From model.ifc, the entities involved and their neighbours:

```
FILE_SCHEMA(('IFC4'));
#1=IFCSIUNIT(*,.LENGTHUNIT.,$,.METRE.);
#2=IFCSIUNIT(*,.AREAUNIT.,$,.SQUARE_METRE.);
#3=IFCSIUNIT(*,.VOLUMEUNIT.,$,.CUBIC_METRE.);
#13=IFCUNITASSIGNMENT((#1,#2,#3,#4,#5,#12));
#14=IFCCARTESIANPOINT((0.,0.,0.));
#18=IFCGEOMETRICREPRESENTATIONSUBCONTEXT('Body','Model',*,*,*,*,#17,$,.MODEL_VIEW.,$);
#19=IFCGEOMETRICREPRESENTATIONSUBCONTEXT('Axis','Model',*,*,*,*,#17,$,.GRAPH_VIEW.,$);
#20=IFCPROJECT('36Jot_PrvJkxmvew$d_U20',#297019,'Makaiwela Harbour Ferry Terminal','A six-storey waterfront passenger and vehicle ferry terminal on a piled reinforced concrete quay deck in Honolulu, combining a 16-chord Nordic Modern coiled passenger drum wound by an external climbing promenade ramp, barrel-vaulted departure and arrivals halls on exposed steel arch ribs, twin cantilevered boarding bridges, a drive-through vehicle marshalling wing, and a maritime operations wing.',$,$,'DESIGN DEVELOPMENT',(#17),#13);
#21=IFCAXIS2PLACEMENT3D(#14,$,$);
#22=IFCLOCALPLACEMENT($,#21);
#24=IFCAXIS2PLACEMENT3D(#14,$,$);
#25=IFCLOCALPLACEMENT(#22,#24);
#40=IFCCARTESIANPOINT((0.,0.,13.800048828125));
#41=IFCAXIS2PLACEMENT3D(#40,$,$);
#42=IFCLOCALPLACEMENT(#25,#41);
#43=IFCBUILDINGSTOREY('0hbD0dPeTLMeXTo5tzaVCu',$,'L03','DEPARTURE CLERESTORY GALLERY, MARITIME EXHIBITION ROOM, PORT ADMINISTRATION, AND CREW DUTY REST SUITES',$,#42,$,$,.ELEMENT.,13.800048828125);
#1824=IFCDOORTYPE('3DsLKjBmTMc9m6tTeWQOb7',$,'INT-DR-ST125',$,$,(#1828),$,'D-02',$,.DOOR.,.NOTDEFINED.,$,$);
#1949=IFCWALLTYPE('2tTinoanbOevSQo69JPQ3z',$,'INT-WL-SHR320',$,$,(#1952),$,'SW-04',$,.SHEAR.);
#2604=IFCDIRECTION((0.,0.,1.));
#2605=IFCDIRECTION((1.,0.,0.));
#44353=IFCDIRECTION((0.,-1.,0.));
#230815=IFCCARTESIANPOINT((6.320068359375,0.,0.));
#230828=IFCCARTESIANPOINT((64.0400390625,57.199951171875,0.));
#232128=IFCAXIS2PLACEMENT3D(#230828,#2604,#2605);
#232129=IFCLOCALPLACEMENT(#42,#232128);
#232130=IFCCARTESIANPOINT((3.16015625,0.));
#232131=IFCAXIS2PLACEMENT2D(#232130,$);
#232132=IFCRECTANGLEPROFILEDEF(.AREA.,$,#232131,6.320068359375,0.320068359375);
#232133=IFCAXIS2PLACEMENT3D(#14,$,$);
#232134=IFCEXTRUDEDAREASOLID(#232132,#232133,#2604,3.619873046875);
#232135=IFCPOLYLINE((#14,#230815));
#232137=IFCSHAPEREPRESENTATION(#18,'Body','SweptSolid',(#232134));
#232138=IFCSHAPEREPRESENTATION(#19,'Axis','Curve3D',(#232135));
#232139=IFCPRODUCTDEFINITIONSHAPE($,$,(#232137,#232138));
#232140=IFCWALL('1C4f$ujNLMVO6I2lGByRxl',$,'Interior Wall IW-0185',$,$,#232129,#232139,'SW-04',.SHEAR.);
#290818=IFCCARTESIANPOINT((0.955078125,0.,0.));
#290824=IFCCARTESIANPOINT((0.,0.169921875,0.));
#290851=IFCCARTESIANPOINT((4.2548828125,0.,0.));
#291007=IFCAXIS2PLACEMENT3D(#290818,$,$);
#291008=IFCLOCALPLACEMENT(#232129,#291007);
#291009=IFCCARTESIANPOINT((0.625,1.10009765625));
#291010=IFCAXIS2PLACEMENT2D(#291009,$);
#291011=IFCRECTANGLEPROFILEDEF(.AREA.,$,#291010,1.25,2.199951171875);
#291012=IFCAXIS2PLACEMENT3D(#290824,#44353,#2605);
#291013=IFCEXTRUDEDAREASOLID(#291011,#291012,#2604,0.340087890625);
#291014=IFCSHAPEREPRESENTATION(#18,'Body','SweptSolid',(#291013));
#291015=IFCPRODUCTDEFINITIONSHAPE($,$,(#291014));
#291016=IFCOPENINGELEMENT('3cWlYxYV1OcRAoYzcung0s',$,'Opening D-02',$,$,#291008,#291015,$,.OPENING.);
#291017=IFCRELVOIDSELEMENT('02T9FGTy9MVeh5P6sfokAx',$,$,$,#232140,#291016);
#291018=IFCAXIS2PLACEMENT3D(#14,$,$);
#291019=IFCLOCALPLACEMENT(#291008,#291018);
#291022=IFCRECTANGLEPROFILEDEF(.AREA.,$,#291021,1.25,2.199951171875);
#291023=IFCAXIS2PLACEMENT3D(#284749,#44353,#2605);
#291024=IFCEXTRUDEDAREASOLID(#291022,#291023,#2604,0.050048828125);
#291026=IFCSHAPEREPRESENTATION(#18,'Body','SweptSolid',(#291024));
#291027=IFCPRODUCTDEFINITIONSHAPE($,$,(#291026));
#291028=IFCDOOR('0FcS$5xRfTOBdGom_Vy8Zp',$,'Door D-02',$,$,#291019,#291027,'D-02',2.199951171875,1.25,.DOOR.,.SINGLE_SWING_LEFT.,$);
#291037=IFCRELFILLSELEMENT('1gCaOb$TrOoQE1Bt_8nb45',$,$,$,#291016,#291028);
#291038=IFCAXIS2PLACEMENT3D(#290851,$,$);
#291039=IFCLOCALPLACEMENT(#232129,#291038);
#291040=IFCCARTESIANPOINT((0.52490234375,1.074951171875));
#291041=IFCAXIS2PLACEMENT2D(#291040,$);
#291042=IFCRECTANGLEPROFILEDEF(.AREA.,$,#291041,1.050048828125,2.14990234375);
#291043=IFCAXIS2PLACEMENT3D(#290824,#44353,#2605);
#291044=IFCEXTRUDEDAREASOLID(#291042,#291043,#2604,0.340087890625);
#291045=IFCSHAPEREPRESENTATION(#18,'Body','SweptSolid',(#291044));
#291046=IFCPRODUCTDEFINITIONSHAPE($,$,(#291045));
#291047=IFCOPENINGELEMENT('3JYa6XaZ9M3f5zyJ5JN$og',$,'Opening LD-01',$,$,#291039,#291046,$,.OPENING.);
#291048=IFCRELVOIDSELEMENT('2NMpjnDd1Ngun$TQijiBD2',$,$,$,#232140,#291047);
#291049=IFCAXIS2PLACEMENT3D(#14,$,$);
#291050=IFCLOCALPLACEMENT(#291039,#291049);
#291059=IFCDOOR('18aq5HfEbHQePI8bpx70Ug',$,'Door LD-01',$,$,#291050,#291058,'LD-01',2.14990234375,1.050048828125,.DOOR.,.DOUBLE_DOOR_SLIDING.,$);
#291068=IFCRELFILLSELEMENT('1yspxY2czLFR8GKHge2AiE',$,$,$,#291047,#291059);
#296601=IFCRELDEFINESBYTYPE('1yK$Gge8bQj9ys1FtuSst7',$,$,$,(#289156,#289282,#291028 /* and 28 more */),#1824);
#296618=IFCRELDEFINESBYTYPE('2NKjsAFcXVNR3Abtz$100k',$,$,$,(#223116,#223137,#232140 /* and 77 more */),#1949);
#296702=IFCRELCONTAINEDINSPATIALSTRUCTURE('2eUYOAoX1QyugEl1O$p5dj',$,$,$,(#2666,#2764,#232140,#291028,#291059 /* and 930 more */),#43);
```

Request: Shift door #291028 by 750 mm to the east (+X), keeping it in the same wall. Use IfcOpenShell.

```python
import ifcopenshell
import ifcopenshell.api.geometry
import ifcopenshell.util.placement

model = ifcopenshell.open("model.ifc")

door = model.by_guid("0FcS$5xRfTOBdGom_Vy8Zp")
opening = door.FillsVoids[0].RelatingOpeningElement
wall = opening.VoidsElements[0].RelatingBuildingElement

wall_matrix = ifcopenshell.util.placement.get_local_placement(wall.ObjectPlacement)
shift = wall_matrix[:3, 0] * 0.75
before = ifcopenshell.util.placement.get_local_placement(door.ObjectPlacement)[:3, 3].copy()

# The door is placed relative to its opening, so it follows when the opening moves.
matrix = ifcopenshell.util.placement.get_local_placement(opening.ObjectPlacement)
matrix[:3, 3] += shift
ifcopenshell.api.geometry.edit_object_placement(
    model, product=opening, matrix=matrix, is_si=False, should_transform_children=True
)

after = ifcopenshell.util.placement.get_local_placement(door.ObjectPlacement)[:3, 3]
print("door moved by", (after - before).round(3) + 0.0)

model.write("model_v2.ifc")
```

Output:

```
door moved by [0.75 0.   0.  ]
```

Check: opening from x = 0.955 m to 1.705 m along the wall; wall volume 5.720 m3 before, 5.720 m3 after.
